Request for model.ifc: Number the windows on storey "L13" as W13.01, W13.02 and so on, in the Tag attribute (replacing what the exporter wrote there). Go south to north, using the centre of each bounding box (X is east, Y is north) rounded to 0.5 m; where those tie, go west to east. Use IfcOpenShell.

First a look at what the model holds.

```python
import ifcopenshell
import ifcopenshell.util.element
import ifcopenshell.util.placement

model = ifcopenshell.open("model.ifc")
print(model.schema)
storey = next(s for s in model.by_type("IfcBuildingStorey") if s.Name == "L13")
windows = [e for e in ifcopenshell.util.element.get_decomposition(storey) if e.is_a("IfcWindow")]
for e in sorted(windows, key=lambda e: e.id()):
    origin = ifcopenshell.util.placement.get_local_placement(e.ObjectPlacement)[:3, 3]
    print(e.id(), e.Tag, e.Name, origin.round(2) + 0.0, sep=" | ")
```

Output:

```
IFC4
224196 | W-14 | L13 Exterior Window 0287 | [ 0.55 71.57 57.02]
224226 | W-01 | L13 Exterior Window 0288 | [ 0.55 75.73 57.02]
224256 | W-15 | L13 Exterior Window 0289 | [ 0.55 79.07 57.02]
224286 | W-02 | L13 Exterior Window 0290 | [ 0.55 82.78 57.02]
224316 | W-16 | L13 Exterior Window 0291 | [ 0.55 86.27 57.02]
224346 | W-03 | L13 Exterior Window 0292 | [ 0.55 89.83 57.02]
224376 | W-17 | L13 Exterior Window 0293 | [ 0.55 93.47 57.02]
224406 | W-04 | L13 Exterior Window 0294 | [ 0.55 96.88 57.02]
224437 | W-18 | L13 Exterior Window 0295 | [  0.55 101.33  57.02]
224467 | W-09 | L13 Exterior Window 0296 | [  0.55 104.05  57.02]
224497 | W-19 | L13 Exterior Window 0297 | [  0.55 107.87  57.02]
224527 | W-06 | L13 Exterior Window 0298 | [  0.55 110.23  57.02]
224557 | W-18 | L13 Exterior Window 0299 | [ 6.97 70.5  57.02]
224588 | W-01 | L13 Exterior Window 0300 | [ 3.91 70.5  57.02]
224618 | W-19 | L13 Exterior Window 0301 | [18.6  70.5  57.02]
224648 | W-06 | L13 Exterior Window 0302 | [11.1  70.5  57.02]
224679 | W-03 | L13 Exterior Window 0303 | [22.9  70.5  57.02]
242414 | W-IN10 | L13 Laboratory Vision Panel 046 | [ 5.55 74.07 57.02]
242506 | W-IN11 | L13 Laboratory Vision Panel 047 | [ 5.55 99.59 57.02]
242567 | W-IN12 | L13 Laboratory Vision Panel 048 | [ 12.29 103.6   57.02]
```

```python
import ifcopenshell
import ifcopenshell.geom
import ifcopenshell.util.element
import ifcopenshell.util.shape

model = ifcopenshell.open("model.ifc")
settings = ifcopenshell.geom.settings()
settings.set("use-world-coords", True)


def centre(element):
    shape = ifcopenshell.geom.create_shape(settings, element)
    return ifcopenshell.util.shape.get_bbox_centroid(shape.geometry)


storey = next(s for s in model.by_type("IfcBuildingStorey") if s.Name == "L13")
windows = [e for e in ifcopenshell.util.element.get_decomposition(storey) if e.is_a("IfcWindow")]

# Insertion points can sit at a corner or the storey origin, so sort by the geometry (in metres).
centres = {e: centre(e) for e in windows}
windows.sort(key=lambda e: (round(centres[e][1] / 0.5), centres[e][0]))

for i, e in enumerate(windows, start=1):
    number = f"W13.{i:02d}"
    e.Tag = number
    print(e.id(), number)

model.write("model-out.ifc")
```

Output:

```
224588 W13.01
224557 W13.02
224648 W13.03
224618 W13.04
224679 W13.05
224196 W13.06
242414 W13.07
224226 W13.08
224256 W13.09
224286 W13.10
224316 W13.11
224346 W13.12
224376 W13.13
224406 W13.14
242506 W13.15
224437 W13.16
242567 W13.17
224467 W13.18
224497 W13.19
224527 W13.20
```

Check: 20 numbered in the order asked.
